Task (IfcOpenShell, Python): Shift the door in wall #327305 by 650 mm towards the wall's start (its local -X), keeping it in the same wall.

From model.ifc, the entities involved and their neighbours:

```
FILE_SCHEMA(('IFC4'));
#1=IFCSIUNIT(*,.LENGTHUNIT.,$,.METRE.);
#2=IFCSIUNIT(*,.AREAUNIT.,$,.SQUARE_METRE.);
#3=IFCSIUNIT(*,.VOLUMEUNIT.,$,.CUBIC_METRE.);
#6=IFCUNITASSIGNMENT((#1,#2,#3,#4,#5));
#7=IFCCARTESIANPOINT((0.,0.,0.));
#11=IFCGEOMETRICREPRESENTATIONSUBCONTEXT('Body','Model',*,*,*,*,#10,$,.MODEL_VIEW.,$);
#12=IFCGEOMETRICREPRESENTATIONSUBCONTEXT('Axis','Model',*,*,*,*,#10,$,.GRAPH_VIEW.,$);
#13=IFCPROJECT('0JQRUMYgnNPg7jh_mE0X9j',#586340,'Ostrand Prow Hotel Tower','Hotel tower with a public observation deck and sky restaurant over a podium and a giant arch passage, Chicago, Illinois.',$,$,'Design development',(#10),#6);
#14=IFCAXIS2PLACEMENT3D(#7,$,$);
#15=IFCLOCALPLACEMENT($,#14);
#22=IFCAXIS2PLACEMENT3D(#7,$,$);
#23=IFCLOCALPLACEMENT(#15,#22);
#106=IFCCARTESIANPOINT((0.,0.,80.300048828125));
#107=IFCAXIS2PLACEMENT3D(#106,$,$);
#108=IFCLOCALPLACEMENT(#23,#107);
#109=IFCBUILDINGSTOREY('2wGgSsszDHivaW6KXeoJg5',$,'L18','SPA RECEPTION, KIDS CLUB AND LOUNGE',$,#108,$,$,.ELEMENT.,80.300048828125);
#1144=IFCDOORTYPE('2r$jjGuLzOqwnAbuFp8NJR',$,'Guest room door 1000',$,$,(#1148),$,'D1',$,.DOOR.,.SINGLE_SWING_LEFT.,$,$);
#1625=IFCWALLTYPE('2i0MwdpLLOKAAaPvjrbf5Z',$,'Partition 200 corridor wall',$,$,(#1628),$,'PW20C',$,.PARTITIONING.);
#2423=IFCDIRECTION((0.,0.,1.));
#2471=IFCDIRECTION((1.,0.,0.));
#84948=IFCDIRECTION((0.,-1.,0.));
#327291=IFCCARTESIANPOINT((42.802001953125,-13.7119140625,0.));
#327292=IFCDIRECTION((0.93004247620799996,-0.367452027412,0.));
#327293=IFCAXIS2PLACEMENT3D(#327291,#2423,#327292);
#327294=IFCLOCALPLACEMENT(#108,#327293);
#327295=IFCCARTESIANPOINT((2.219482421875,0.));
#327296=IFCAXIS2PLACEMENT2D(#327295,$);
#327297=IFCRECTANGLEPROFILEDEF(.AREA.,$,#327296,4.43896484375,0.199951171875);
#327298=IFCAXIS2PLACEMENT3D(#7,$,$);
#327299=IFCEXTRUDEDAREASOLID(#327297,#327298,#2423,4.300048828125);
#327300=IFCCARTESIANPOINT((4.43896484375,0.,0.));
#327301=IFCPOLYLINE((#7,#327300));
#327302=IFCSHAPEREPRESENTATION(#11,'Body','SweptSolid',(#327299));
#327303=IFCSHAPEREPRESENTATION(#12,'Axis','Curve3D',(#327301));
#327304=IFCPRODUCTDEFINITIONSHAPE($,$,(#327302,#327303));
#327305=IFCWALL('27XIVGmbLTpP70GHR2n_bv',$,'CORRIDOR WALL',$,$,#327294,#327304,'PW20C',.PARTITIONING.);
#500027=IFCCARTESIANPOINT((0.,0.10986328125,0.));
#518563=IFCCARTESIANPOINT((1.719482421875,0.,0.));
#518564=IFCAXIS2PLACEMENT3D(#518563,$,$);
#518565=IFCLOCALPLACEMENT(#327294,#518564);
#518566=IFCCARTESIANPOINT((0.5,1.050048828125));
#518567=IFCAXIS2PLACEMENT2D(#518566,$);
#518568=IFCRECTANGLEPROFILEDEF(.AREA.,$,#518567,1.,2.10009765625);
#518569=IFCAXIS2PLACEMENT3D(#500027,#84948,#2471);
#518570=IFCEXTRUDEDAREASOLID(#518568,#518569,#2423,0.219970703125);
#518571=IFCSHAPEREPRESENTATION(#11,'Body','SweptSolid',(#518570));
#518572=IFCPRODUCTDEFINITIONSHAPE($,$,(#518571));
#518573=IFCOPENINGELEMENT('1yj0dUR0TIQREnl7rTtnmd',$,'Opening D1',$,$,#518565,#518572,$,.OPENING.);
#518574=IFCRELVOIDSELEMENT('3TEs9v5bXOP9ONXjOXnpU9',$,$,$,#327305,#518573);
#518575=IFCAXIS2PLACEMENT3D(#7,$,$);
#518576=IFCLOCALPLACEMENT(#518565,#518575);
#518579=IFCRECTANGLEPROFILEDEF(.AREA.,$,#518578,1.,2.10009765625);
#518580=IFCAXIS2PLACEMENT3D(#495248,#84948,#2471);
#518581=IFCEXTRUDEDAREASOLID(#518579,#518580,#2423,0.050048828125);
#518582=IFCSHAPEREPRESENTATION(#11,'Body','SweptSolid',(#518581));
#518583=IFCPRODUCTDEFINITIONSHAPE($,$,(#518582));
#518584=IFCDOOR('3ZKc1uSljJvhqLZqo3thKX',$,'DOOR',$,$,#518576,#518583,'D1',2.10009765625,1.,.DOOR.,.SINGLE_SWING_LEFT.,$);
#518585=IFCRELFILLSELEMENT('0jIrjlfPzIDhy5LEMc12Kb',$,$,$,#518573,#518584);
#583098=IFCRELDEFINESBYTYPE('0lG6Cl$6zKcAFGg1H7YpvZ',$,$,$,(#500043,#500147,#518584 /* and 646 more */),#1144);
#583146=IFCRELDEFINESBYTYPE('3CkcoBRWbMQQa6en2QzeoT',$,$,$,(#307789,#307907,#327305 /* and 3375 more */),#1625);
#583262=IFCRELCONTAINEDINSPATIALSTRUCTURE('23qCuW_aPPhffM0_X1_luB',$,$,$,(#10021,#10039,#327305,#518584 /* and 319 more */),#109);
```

```python
import ifcopenshell
import ifcopenshell.api.geometry
import ifcopenshell.util.placement

model = ifcopenshell.open("model.ifc")

door = model.by_guid("3ZKc1uSljJvhqLZqo3thKX")
opening = door.FillsVoids[0].RelatingOpeningElement
wall = opening.VoidsElements[0].RelatingBuildingElement

wall_matrix = ifcopenshell.util.placement.get_local_placement(wall.ObjectPlacement)
shift = wall_matrix[:3, 0] * -0.65
before = ifcopenshell.util.placement.get_local_placement(door.ObjectPlacement)[:3, 3].copy()

# The door is placed relative to its opening, so it follows when the opening moves.
matrix = ifcopenshell.util.placement.get_local_placement(opening.ObjectPlacement)
matrix[:3, 3] += shift
ifcopenshell.api.geometry.edit_object_placement(
    model, product=opening, matrix=matrix, is_si=False, should_transform_children=True
)

after = ifcopenshell.util.placement.get_local_placement(door.ObjectPlacement)[:3, 3]
print("door moved by", (after - before).round(3) + 0.0)

model.write("model_updated.ifc")
```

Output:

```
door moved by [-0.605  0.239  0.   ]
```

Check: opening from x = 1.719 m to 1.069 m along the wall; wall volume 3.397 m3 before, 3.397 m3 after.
